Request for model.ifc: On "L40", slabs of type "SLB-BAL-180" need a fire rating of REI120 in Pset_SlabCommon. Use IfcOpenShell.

First a look at what the model holds.

```python
import ifcopenshell
import ifcopenshell.util.element

model = ifcopenshell.open("model.ifc")
print(model.schema)
storey = next(s for s in model.by_type("IfcBuildingStorey") if s.Name == "L40")
slabs = [e for e in ifcopenshell.util.element.get_decomposition(storey) if e.is_a("IfcSlab")]
seen = {}
for e in slabs:
    element_type = ifcopenshell.util.element.get_type(e)
    key = (element_type.Name if element_type != e and element_type else None, ifcopenshell.util.element.get_pset(e, "Pset_SlabCommon", "FireRating"))
    seen[key] = seen.get(key, 0) + 1
for (name, value), count in sorted(seen.items(), key=str):
    print(count, "x", name, "|", value)
```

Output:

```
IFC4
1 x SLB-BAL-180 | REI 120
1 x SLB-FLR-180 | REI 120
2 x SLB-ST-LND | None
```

```python
import ifcopenshell
import ifcopenshell.api.pset
import ifcopenshell.util.element

model = ifcopenshell.open("model.ifc")

storey = next(s for s in model.by_type("IfcBuildingStorey") if s.Name == "L40")
slabs = [e for e in ifcopenshell.util.element.get_decomposition(storey) if e.is_a("IfcSlab")]

count = 0
for e in slabs:
    element_type = ifcopenshell.util.element.get_type(e)
    if element_type in (None, e) or element_type.Name != "SLB-BAL-180":
        continue
    found = ifcopenshell.util.element.get_pset(e, "Pset_SlabCommon", should_inherit=False)
    if found:
        pset = model.by_id(found["id"])
        if len(ifcopenshell.util.element.get_elements_by_pset(pset)) > 1:
            pset = ifcopenshell.api.pset.unshare_pset(model, products=[e], pset=pset)[0]
    else:
        pset = ifcopenshell.api.pset.add_pset(model, product=e, name="Pset_SlabCommon")
    ifcopenshell.api.pset.edit_pset(model, pset=pset, properties={"FireRating": "REI120"})
    count += 1

print(count, "slabs updated")

model.write("model_rev.ifc")
```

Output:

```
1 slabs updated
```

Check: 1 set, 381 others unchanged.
